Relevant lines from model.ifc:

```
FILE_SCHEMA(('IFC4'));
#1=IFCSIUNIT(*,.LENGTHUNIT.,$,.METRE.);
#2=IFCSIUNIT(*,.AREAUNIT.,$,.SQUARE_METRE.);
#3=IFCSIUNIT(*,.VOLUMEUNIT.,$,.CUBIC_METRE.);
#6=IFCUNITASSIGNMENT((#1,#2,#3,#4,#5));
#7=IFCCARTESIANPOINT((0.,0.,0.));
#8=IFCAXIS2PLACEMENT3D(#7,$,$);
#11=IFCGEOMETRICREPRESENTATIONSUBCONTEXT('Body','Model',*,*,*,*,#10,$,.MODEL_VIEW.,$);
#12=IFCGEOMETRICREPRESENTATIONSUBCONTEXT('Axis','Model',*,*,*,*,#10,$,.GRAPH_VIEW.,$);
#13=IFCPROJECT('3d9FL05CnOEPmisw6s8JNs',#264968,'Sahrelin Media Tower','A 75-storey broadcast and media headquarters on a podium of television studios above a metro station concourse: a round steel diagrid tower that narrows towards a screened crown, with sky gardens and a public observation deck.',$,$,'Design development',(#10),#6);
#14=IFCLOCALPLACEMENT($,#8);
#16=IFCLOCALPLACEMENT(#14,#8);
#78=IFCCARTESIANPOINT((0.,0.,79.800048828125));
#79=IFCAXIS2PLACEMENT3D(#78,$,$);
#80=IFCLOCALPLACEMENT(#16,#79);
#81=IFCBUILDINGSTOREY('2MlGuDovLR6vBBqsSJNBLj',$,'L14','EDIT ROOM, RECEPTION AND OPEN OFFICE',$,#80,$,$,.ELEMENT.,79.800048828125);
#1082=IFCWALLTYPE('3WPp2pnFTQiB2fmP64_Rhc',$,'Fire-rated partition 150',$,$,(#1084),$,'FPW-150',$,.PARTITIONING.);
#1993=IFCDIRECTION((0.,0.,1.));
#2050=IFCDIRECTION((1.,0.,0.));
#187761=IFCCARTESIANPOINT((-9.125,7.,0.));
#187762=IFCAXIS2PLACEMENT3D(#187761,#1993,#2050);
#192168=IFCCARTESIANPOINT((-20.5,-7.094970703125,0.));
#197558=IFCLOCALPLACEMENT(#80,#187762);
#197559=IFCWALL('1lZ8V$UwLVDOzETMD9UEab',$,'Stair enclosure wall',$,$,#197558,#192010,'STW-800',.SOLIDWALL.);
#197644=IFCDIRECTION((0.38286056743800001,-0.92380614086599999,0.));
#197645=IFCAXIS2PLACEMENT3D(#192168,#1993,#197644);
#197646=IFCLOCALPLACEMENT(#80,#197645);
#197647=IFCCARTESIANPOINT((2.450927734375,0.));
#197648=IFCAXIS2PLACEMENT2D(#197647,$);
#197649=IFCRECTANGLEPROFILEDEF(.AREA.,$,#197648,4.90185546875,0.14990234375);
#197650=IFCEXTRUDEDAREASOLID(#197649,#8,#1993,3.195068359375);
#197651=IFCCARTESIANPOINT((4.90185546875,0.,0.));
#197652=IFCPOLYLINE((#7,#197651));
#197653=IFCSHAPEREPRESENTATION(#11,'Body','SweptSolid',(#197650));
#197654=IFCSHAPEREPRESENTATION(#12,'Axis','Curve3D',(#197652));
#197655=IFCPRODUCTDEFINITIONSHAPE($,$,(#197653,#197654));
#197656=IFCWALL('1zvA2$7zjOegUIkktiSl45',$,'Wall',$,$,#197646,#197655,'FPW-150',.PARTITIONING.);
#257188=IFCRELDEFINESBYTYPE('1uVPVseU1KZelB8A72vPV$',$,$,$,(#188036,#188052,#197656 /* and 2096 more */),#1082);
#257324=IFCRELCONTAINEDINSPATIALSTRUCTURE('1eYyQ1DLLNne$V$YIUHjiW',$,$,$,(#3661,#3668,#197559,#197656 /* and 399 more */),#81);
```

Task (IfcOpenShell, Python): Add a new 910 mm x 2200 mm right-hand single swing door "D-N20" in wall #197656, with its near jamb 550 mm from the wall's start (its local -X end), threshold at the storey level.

```python
import numpy as np
import ifcopenshell
import ifcopenshell.api.feature
import ifcopenshell.api.geometry
import ifcopenshell.api.root
import ifcopenshell.api.spatial
import ifcopenshell.geom
import ifcopenshell.util.element
import ifcopenshell.util.placement
import ifcopenshell.util.representation
import ifcopenshell.util.shape
import ifcopenshell.util.unit

model = ifcopenshell.open("model.ifc")
unit_scale = ifcopenshell.util.unit.calculate_unit_scale(model)
settings = ifcopenshell.geom.settings()


def volume(element):
    """Net volume in cubic metres, openings subtracted."""
    shape = ifcopenshell.geom.create_shape(settings, element)
    return ifcopenshell.util.shape.get_volume(shape.geometry)


wall = model.by_id(197656)
storey = ifcopenshell.util.element.get_container(wall, ifc_class="IfcBuildingStorey")
context = ifcopenshell.util.representation.get_context(model, "Model", "Body", "MODEL_VIEW")
before = volume(wall)

width, height, from_end, sill = 0.91, 2.2, 0.55, 0.0  # metres

# The wall runs along its own X axis, and the end named is its -X end.
wall_shape = ifcopenshell.geom.create_shape(settings, wall)
x, y, z = ifcopenshell.util.shape.get_vertices(wall_shape.geometry).T
start = x.min() + from_end
face, thickness = float(y.min()), float(y.max() - y.min())
wall_matrix = ifcopenshell.util.placement.get_local_placement(wall.ObjectPlacement)
level = ifcopenshell.util.placement.get_local_placement(storey.ObjectPlacement)[2, 3]


def in_wall(x, y):
    """Placement at x, y metres in the wall's axes, at sill height."""
    matrix = wall_matrix.copy()
    matrix[:, 3] = wall_matrix @ np.array([x / unit_scale, y / unit_scale, 0.0, 1.0])
    matrix[2, 3] = level + sill / unit_scale
    return matrix


# Opening: a box that overshoots both wall faces by 50 mm.
opening = ifcopenshell.api.root.create_entity(model, ifc_class="IfcOpeningElement", predefined_type="OPENING")
box = ifcopenshell.api.geometry.add_wall_representation(
    model, context=context, length=width, height=height, thickness=thickness + 0.1
)
ifcopenshell.api.geometry.assign_representation(model, product=opening, representation=box)
ifcopenshell.api.geometry.edit_object_placement(model, product=opening, matrix=in_wall(start, face - 0.05), is_si=False)
ifcopenshell.api.feature.add_feature(model, feature=opening, element=wall)

door = ifcopenshell.api.root.create_entity(model, ifc_class="IfcDoor", name="D-N20", predefined_type="DOOR")
door.OverallWidth, door.OverallHeight = width / unit_scale, height / unit_scale
door.OperationType = "SINGLE_SWING_RIGHT"
body = ifcopenshell.api.geometry.add_door_representation(
    model,
    context=context,
    overall_width=door.OverallWidth,
    overall_height=door.OverallHeight,
    operation_type="SINGLE_SWING_RIGHT",
    lining_properties={"LiningDepth": thickness / unit_scale, "ThresholdDepth": thickness / unit_scale},
)
ifcopenshell.api.geometry.assign_representation(model, product=door, representation=body)
ifcopenshell.api.spatial.assign_container(model, products=[door], relating_structure=storey)
ifcopenshell.api.feature.add_filling(model, opening=opening, element=door)

# The lining spans the wall, so the door starts at the wall face.
ifcopenshell.api.geometry.edit_object_placement(model, product=door, matrix=in_wall(start, face), is_si=False)

after = volume(wall)

print(f"wall volume {before:.3f} -> {after:.3f} m3")

model.write("model_updated.ifc")
```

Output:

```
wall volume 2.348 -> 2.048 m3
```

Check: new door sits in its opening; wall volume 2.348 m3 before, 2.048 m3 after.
